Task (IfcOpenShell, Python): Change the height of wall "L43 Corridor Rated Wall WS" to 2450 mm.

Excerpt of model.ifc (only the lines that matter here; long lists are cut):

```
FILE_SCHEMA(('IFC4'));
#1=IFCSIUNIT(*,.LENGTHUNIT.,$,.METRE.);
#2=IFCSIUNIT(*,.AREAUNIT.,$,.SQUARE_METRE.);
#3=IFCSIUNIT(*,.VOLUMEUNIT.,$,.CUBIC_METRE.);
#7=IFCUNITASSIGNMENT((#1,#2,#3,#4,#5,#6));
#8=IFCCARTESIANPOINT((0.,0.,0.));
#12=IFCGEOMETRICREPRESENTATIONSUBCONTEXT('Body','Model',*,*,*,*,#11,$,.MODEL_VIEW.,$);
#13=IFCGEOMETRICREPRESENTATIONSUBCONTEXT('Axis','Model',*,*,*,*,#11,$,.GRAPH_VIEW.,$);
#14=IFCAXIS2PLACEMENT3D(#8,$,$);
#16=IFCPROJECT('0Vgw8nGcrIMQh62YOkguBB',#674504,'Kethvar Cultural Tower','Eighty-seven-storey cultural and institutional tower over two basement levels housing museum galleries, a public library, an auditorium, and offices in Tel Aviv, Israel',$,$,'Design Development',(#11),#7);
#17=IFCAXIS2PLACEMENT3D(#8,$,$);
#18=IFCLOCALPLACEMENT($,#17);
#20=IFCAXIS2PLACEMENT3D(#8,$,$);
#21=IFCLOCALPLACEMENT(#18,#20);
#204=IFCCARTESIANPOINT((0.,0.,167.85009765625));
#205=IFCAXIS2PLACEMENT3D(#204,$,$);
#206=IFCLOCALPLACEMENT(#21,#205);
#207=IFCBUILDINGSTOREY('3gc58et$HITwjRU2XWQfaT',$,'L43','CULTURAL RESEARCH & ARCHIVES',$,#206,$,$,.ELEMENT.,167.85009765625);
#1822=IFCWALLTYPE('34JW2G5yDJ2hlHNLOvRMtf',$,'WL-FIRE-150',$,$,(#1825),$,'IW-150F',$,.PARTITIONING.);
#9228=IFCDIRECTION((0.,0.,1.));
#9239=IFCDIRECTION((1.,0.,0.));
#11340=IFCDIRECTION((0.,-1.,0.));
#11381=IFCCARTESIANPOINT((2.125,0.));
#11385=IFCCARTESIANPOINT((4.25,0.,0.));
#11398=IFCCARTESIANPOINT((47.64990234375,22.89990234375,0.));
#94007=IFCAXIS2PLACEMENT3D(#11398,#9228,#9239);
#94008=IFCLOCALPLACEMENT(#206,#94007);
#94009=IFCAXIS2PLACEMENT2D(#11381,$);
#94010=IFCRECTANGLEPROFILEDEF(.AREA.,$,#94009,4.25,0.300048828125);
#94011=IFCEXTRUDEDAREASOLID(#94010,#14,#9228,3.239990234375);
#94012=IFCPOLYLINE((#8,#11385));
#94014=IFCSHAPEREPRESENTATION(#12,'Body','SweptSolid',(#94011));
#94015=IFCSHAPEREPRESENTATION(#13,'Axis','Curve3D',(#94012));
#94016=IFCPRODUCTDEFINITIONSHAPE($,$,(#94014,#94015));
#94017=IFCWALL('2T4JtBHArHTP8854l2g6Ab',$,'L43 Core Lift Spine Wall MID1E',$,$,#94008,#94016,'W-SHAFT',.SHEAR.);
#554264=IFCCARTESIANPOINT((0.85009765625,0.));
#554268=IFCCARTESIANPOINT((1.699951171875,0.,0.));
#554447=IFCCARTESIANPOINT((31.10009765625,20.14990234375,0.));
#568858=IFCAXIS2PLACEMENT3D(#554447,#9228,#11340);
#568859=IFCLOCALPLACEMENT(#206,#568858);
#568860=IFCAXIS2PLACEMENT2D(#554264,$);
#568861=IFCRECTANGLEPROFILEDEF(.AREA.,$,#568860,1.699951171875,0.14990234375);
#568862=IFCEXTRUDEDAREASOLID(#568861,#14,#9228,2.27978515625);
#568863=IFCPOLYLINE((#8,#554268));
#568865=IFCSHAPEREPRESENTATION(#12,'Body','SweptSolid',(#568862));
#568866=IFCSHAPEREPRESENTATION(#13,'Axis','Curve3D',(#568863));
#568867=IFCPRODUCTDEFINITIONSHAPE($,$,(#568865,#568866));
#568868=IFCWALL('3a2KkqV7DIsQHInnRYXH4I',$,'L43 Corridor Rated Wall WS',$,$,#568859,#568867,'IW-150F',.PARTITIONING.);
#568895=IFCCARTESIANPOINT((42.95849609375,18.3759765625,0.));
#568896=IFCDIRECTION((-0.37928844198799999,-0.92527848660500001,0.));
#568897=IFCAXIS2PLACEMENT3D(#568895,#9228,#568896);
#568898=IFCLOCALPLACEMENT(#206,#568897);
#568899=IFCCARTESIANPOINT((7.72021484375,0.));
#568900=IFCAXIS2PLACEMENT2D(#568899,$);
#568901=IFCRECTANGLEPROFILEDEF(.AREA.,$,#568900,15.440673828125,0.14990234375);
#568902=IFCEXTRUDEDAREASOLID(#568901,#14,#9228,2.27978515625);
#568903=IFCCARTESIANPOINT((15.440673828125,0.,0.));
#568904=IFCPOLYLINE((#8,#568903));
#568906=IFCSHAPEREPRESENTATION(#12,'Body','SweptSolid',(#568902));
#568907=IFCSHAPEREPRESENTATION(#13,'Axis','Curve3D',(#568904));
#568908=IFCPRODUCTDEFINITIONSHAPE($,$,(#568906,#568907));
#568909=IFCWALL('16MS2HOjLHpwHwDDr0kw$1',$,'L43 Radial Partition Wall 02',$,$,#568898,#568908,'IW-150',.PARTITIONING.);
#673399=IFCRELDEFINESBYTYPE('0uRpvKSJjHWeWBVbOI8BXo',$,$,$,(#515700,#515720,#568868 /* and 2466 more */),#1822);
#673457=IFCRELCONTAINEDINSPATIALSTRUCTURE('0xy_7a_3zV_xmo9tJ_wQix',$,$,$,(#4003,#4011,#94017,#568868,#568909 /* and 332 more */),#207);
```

```python
import ifcopenshell
import ifcopenshell.geom
import ifcopenshell.util.representation
import ifcopenshell.util.shape
import ifcopenshell.util.unit

model = ifcopenshell.open("model.ifc")
unit_scale = ifcopenshell.util.unit.calculate_unit_scale(model)
settings = ifcopenshell.geom.settings()


def volume(element):
    """Net volume in cubic metres, openings subtracted."""
    shape = ifcopenshell.geom.create_shape(settings, element)
    return ifcopenshell.util.shape.get_volume(shape.geometry)


wall = model.by_guid("3a2KkqV7DIsQHInnRYXH4I")
before = volume(wall)

body = ifcopenshell.util.representation.get_representation(wall, "Model", "Body")
solid = body.Items[0]
old_height = solid.Depth
solid.Depth = 2.45 / unit_scale
after = volume(wall)

print(f"height {old_height:g} -> {solid.Depth:g}, volume {before:.3f} -> {after:.3f} m3")

model.write("model_rev.ifc")
```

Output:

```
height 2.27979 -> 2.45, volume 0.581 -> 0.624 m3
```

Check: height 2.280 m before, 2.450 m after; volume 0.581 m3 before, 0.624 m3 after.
